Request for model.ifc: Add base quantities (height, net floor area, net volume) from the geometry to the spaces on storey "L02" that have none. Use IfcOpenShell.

First a look at what the model holds.

```python
import ifcopenshell
import ifcopenshell.util.element
import ifcopenshell.util.unit

model = ifcopenshell.open("model.ifc")
print(model.schema)
for unit_type in ("LENGTHUNIT", "AREAUNIT", "VOLUMEUNIT"):
    print(unit_type, ifcopenshell.util.unit.calculate_unit_scale(model, unit_type))
storey = next(s for s in model.by_type("IfcBuildingStorey") if s.Name == "L02")
spaces = [e for e in ifcopenshell.util.element.get_decomposition(storey) if e.is_a("IfcSpace")]
for e in sorted(spaces, key=lambda e: e.id()):
    print(e.id(), e.is_a(), e.Name, list(ifcopenshell.util.element.get_psets(e, qtos_only=True)), sep=" | ")
```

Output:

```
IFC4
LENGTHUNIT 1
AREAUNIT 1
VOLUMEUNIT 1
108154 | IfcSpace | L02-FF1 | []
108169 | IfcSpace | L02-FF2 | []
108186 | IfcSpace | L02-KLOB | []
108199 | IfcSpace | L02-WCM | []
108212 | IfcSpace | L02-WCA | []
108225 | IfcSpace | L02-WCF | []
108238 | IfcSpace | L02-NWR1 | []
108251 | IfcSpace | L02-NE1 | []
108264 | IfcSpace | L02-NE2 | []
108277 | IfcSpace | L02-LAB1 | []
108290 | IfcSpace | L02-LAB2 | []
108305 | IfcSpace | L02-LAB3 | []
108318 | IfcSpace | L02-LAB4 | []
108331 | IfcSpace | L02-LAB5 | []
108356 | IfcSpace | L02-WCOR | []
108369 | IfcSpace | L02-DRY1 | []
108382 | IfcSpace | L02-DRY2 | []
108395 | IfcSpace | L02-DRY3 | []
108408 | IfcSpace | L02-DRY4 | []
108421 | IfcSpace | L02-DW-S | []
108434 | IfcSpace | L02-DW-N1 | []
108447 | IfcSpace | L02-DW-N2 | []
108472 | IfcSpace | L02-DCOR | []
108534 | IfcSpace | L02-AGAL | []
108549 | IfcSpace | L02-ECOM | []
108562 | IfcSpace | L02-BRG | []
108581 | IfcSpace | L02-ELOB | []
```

```python
import ifcopenshell
import ifcopenshell.api.pset
import ifcopenshell.geom
import ifcopenshell.util.element
import ifcopenshell.util.shape
import ifcopenshell.util.unit

model = ifcopenshell.open("model.ifc")
unit_scale = ifcopenshell.util.unit.calculate_unit_scale(model)
area_scale = ifcopenshell.util.unit.calculate_unit_scale(model, "AREAUNIT")
volume_scale = ifcopenshell.util.unit.calculate_unit_scale(model, "VOLUMEUNIT")
settings = ifcopenshell.geom.settings()

storey = next(s for s in model.by_type("IfcBuildingStorey") if s.Name == "L02")
spaces = [e for e in ifcopenshell.util.element.get_decomposition(storey) if e.is_a("IfcSpace")]

for e in sorted(spaces, key=lambda e: e.id()):
    if ifcopenshell.util.element.get_psets(e, qtos_only=True, should_inherit=False):
        continue
    # Geometry comes back in metres, in the element's own axes.
    shape = ifcopenshell.geom.create_shape(settings, e)
    values = {
        "Height": ifcopenshell.util.shape.get_z(shape.geometry) / unit_scale,
        "NetFloorArea": ifcopenshell.util.shape.get_footprint_area(shape.geometry) / area_scale,
        "NetVolume": ifcopenshell.util.shape.get_volume(shape.geometry) / volume_scale,
    }
    qto = ifcopenshell.api.pset.add_qto(model, product=e, name="Qto_SpaceBaseQuantities")
    ifcopenshell.api.pset.edit_qto(model, qto=qto, properties=values)
    print(e.id(), {k: round(v, 3) for k, v in values.items()})

model.write("model_edited.ifc")
```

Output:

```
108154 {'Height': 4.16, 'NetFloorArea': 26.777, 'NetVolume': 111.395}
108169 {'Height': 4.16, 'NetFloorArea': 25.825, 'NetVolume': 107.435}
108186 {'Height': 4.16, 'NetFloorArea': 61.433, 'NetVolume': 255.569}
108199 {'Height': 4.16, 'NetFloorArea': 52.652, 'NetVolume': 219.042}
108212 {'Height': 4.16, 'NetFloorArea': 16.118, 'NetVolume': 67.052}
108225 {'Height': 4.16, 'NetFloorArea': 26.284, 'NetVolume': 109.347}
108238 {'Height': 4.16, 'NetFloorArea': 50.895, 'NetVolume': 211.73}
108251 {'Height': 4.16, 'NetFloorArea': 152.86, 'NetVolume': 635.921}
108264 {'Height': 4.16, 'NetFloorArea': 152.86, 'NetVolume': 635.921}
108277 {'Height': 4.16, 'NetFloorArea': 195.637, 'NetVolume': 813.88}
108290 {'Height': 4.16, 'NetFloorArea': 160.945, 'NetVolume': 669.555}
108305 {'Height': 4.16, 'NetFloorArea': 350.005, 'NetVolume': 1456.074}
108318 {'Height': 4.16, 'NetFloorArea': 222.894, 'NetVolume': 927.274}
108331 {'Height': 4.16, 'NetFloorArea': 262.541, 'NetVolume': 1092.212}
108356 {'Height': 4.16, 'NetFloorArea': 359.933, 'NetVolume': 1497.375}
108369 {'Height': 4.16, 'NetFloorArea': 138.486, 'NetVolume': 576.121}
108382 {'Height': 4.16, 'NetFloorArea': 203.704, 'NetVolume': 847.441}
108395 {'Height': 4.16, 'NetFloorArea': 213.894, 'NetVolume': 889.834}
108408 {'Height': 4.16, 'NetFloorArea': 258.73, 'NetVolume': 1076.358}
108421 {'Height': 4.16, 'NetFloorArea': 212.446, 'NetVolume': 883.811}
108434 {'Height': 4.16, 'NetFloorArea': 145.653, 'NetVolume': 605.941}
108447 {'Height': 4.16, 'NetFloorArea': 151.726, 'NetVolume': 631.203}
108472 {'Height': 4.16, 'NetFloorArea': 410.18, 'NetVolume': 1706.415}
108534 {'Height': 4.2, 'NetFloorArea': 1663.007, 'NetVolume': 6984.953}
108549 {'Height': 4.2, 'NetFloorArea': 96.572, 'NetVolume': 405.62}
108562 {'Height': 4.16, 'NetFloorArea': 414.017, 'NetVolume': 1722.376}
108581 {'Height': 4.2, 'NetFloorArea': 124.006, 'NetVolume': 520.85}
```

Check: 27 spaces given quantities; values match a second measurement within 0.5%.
